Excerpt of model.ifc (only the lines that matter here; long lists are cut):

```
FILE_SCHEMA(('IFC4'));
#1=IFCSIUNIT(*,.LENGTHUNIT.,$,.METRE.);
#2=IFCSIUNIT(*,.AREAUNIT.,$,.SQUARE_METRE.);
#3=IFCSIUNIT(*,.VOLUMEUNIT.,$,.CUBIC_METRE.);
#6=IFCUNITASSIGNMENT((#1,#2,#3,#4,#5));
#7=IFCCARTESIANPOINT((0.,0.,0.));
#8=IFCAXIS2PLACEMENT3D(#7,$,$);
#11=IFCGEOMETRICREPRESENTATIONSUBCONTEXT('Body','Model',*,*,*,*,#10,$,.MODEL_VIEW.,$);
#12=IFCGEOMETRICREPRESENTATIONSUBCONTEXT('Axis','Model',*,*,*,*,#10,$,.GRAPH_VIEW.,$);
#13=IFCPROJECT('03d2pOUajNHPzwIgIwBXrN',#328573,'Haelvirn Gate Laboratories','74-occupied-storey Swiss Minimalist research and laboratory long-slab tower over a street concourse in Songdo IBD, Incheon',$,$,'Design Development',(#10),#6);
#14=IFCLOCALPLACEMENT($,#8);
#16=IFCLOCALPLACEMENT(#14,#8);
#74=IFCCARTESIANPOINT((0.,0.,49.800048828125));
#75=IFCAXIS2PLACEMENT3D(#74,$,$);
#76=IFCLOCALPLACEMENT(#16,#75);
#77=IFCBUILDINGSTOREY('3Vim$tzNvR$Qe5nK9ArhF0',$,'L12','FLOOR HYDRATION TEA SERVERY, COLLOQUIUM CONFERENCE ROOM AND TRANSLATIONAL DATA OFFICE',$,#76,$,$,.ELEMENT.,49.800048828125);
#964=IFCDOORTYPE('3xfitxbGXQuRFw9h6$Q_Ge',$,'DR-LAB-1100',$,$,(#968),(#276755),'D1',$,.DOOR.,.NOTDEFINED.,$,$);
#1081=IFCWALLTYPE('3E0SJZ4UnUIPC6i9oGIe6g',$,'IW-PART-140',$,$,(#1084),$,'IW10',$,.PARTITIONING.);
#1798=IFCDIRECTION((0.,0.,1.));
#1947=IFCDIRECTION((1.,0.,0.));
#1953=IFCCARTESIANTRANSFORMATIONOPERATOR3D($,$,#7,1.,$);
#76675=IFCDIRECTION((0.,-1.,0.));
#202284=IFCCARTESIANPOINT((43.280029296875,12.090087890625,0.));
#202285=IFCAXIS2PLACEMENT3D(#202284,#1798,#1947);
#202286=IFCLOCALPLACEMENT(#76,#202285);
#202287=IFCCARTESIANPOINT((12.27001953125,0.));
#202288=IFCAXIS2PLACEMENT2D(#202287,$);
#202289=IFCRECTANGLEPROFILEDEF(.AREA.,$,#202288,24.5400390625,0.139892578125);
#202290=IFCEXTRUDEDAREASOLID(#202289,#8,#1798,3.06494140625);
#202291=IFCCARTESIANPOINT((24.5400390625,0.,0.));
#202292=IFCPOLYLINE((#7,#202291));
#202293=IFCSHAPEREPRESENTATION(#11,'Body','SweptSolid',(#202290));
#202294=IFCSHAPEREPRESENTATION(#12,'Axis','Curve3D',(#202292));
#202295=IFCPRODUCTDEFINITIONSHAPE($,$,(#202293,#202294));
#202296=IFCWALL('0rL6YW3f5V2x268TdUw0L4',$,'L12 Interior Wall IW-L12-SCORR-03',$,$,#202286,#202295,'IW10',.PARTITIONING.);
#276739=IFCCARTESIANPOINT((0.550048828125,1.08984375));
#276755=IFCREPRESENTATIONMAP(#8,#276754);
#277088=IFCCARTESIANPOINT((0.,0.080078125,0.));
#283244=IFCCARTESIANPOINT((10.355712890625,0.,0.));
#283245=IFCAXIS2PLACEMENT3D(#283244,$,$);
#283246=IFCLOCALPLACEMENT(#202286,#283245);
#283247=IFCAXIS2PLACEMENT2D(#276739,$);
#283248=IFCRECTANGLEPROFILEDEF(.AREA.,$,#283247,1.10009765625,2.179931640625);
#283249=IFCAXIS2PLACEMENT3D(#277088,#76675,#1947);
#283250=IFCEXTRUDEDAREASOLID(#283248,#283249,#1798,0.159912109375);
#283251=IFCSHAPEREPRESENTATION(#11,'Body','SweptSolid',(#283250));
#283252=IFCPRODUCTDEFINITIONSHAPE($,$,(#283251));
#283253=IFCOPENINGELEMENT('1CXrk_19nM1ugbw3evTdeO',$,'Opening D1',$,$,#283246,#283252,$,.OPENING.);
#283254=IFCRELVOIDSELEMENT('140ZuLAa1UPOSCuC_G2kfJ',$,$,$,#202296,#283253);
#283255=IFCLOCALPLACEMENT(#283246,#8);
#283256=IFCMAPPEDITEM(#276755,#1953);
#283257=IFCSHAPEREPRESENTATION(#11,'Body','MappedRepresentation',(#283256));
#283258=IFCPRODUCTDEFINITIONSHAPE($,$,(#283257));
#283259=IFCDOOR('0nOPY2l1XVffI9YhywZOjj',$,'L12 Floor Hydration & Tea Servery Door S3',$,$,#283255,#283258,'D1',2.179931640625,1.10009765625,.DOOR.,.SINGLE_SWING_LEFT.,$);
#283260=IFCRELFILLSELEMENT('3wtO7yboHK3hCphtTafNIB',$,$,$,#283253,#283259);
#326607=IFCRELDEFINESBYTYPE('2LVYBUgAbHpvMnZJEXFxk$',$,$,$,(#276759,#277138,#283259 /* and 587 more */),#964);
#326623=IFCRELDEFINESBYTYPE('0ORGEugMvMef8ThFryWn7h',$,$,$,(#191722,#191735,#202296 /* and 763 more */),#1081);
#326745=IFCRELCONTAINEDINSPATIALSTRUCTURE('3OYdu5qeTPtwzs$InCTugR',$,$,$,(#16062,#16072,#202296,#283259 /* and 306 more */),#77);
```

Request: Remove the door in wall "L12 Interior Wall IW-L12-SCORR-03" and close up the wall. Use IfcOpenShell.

```python
import ifcopenshell
import ifcopenshell.api.feature
import ifcopenshell.api.root
import ifcopenshell.geom
import ifcopenshell.util.shape

model = ifcopenshell.open("model.ifc")
settings = ifcopenshell.geom.settings()


def volume(element):
    """Net volume in cubic metres, openings subtracted."""
    shape = ifcopenshell.geom.create_shape(settings, element)
    return ifcopenshell.util.shape.get_volume(shape.geometry)


door = model.by_id(283259)
opening = door.FillsVoids[0].RelatingOpeningElement
wall = opening.VoidsElements[0].RelatingBuildingElement
before = volume(wall)

ifcopenshell.api.root.remove_product(model, product=door)
ifcopenshell.api.feature.remove_feature(model, feature=opening)

after = volume(wall)

print(f"wall volume {before:.3f} -> {after:.3f} m3")

model.write("model_updated.ifc")
```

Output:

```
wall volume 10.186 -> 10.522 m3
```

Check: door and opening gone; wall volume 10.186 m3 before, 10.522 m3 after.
